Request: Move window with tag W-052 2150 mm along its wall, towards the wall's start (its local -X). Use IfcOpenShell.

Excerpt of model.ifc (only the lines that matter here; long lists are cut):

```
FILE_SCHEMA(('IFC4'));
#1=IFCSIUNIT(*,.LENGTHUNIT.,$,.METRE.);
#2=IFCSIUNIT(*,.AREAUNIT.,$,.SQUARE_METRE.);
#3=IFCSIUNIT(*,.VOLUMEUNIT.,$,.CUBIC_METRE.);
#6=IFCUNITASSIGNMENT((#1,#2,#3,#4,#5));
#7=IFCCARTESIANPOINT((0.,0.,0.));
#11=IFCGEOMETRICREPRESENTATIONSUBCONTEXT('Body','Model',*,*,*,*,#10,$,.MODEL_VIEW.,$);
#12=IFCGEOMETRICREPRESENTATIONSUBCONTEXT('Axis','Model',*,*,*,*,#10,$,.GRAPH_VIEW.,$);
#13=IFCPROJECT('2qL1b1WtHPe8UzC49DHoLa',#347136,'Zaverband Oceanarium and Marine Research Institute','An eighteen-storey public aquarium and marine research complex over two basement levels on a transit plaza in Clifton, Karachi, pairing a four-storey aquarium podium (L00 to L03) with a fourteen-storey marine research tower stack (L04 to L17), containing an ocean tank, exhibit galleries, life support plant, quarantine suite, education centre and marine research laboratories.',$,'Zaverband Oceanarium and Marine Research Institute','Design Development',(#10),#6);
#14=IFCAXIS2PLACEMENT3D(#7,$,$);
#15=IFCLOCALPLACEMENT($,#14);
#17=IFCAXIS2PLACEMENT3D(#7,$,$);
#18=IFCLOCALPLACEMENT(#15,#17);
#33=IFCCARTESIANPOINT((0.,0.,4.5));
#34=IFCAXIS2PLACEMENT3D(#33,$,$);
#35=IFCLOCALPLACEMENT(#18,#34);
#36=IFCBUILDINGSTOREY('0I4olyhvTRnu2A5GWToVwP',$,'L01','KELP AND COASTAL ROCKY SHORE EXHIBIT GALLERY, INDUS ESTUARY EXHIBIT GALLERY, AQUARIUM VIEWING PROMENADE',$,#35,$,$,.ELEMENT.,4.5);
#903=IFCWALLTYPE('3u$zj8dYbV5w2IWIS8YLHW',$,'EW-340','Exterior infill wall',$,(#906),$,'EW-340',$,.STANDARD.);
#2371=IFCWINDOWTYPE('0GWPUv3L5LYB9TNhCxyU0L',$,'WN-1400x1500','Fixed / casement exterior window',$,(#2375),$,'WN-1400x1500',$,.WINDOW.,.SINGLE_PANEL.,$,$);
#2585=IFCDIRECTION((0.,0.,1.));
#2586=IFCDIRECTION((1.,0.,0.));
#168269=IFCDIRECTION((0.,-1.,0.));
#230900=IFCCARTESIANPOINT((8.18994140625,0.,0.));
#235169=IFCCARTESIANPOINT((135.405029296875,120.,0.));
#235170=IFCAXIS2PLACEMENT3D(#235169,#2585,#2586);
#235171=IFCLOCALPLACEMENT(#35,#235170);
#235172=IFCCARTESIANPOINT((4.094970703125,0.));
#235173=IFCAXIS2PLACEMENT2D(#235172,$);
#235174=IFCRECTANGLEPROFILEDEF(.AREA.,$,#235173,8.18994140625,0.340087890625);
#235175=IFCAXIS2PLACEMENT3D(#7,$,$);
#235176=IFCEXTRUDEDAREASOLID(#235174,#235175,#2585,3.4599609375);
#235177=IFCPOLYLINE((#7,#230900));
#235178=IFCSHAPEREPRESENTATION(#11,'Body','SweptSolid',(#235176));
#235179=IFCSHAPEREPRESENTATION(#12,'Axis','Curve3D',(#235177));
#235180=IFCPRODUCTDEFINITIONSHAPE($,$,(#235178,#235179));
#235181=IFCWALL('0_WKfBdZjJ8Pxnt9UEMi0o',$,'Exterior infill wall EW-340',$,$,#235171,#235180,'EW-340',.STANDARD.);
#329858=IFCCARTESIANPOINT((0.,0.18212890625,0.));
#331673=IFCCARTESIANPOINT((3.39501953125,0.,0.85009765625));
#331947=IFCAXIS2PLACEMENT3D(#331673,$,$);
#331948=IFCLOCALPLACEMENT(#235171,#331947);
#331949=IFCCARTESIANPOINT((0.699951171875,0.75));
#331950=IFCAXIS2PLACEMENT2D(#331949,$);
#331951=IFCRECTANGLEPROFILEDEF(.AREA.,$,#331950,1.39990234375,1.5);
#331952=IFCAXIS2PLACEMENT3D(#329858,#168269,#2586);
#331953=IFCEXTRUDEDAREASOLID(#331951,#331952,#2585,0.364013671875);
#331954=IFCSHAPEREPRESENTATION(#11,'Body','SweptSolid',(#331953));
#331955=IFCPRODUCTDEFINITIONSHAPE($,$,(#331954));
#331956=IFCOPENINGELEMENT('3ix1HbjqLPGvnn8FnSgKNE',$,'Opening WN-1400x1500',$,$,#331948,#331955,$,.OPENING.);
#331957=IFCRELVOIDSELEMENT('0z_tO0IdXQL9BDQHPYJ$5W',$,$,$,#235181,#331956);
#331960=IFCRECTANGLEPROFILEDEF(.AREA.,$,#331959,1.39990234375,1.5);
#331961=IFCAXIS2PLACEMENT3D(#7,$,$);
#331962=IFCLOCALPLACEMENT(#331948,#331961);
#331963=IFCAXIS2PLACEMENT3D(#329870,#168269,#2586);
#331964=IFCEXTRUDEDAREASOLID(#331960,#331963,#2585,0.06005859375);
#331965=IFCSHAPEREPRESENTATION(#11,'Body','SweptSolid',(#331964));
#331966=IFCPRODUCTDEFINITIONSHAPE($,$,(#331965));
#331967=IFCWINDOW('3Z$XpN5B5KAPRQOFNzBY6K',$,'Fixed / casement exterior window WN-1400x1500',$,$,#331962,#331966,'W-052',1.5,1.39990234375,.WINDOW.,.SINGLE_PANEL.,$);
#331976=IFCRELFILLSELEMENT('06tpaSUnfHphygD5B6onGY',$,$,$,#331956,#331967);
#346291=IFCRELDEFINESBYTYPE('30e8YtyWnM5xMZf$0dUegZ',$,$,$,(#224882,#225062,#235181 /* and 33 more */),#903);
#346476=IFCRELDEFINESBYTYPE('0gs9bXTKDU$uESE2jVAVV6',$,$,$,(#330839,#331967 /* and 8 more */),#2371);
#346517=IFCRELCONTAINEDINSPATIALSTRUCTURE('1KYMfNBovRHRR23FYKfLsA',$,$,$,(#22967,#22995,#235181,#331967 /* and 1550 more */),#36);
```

```python
import ifcopenshell
import ifcopenshell.api.geometry
import ifcopenshell.util.placement
import ifcopenshell.util.unit

model = ifcopenshell.open("model.ifc")
unit_scale = ifcopenshell.util.unit.calculate_unit_scale(model)

window = model.by_guid("3Z$XpN5B5KAPRQOFNzBY6K")
opening = window.FillsVoids[0].RelatingOpeningElement
wall = opening.VoidsElements[0].RelatingBuildingElement

wall_matrix = ifcopenshell.util.placement.get_local_placement(wall.ObjectPlacement)
shift = wall_matrix[:3, 0] * -2.15 / unit_scale
before = ifcopenshell.util.placement.get_local_placement(window.ObjectPlacement)[:3, 3].copy()

# The window is placed relative to its opening, so it follows when the opening moves.
matrix = ifcopenshell.util.placement.get_local_placement(opening.ObjectPlacement)
matrix[:3, 3] += shift
ifcopenshell.api.geometry.edit_object_placement(
    model, product=opening, matrix=matrix, is_si=False, should_transform_children=True
)

after = ifcopenshell.util.placement.get_local_placement(window.ObjectPlacement)[:3, 3]
print("window moved by", (after - before).round(3) + 0.0)

model.write("model_updated.ifc")
```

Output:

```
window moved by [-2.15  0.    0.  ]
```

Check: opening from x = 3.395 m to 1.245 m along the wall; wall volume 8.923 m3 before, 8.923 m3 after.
